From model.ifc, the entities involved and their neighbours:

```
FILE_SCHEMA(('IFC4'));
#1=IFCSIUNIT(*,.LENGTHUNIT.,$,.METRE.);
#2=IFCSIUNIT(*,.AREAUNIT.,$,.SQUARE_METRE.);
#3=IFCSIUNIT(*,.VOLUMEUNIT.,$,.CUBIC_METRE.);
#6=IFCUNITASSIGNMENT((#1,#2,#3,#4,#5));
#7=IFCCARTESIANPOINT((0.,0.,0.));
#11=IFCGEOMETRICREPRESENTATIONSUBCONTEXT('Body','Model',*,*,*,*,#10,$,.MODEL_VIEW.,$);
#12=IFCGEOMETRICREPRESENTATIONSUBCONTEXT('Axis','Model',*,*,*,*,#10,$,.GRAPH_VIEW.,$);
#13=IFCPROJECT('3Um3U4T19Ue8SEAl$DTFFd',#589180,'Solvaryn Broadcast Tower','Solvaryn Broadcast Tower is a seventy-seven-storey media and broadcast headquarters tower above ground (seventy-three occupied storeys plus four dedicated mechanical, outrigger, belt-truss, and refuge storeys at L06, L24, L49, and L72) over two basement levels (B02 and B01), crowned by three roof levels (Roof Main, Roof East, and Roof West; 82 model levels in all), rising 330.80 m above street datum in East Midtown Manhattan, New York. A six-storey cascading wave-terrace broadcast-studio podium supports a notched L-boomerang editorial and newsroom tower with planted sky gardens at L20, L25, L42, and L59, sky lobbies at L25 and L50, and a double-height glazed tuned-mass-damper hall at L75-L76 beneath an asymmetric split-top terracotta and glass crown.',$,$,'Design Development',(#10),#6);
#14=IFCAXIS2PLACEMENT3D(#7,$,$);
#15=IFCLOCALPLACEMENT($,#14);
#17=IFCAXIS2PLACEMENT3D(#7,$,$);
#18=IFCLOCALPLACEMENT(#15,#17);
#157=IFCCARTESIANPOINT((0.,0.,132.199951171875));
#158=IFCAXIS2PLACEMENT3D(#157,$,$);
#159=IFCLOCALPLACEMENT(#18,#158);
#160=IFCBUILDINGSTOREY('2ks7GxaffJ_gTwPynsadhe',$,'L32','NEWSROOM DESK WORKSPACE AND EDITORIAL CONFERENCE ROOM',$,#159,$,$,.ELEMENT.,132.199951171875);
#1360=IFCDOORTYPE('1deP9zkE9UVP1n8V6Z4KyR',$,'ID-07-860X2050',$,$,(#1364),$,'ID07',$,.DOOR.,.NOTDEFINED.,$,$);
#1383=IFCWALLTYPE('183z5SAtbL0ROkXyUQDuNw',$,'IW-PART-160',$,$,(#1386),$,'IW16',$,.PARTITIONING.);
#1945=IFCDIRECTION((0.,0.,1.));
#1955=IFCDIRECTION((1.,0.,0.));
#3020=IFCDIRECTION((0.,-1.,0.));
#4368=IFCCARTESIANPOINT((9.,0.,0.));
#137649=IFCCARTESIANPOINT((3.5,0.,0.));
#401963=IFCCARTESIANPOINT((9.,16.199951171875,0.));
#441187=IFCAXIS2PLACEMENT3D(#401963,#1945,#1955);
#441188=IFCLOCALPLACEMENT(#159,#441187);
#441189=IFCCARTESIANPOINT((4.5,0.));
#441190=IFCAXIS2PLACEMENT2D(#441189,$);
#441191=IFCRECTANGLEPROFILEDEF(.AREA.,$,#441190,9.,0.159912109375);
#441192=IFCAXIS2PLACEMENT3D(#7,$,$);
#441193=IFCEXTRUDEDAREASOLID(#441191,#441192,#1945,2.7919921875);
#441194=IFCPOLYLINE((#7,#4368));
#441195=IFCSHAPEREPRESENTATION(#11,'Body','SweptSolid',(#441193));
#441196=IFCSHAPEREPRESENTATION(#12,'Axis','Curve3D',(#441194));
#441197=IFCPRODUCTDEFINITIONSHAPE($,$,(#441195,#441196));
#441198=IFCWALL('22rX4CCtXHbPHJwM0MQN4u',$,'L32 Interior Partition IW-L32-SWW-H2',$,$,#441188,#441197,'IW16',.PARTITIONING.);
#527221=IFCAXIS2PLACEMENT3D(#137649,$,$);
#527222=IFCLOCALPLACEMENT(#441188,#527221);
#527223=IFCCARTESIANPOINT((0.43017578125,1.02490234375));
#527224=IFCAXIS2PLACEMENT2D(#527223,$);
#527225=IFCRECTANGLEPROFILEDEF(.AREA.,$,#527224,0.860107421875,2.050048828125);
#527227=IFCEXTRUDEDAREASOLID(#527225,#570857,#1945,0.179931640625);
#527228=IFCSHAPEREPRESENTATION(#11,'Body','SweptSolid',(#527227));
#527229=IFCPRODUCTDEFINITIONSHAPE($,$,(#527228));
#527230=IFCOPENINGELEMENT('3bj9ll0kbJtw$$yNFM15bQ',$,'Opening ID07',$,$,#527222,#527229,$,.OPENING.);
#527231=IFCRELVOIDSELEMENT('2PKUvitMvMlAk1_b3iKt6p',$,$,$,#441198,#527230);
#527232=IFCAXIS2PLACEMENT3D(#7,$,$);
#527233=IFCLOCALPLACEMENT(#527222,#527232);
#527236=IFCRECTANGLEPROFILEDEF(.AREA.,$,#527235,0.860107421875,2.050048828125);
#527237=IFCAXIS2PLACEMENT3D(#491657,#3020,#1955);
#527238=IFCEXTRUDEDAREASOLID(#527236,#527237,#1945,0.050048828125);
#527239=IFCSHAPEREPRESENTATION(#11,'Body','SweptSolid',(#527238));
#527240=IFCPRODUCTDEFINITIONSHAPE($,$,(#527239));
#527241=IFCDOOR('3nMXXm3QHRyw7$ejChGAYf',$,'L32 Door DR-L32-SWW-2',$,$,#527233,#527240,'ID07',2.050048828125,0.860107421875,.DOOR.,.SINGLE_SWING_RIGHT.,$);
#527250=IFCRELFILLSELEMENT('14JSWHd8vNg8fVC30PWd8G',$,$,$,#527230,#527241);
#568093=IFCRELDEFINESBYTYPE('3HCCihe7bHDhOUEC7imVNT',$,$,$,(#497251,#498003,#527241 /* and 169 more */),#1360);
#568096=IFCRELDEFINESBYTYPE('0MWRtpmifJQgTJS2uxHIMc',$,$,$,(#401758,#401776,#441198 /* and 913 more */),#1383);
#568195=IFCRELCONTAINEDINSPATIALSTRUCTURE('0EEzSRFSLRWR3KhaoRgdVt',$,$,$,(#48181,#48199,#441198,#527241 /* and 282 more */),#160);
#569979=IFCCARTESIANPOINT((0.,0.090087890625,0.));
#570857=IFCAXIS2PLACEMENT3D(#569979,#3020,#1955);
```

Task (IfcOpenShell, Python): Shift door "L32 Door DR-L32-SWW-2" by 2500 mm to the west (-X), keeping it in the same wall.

```python
import ifcopenshell
import ifcopenshell.api.geometry
import ifcopenshell.util.placement

model = ifcopenshell.open("model.ifc")

door = model.by_guid("3nMXXm3QHRyw7$ejChGAYf")
opening = door.FillsVoids[0].RelatingOpeningElement
wall = opening.VoidsElements[0].RelatingBuildingElement

wall_matrix = ifcopenshell.util.placement.get_local_placement(wall.ObjectPlacement)
shift = wall_matrix[:3, 0] * -2.5
before = ifcopenshell.util.placement.get_local_placement(door.ObjectPlacement)[:3, 3].copy()

# The door is placed relative to its opening, so it follows when the opening moves.
matrix = ifcopenshell.util.placement.get_local_placement(opening.ObjectPlacement)
matrix[:3, 3] += shift
ifcopenshell.api.geometry.edit_object_placement(
    model, product=opening, matrix=matrix, is_si=False, should_transform_children=True
)

after = ifcopenshell.util.placement.get_local_placement(door.ObjectPlacement)[:3, 3]
print("door moved by", (after - before).round(3) + 0.0)

model.write("model-out.ifc")
```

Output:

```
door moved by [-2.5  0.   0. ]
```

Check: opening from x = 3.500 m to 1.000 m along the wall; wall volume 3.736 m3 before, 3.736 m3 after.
